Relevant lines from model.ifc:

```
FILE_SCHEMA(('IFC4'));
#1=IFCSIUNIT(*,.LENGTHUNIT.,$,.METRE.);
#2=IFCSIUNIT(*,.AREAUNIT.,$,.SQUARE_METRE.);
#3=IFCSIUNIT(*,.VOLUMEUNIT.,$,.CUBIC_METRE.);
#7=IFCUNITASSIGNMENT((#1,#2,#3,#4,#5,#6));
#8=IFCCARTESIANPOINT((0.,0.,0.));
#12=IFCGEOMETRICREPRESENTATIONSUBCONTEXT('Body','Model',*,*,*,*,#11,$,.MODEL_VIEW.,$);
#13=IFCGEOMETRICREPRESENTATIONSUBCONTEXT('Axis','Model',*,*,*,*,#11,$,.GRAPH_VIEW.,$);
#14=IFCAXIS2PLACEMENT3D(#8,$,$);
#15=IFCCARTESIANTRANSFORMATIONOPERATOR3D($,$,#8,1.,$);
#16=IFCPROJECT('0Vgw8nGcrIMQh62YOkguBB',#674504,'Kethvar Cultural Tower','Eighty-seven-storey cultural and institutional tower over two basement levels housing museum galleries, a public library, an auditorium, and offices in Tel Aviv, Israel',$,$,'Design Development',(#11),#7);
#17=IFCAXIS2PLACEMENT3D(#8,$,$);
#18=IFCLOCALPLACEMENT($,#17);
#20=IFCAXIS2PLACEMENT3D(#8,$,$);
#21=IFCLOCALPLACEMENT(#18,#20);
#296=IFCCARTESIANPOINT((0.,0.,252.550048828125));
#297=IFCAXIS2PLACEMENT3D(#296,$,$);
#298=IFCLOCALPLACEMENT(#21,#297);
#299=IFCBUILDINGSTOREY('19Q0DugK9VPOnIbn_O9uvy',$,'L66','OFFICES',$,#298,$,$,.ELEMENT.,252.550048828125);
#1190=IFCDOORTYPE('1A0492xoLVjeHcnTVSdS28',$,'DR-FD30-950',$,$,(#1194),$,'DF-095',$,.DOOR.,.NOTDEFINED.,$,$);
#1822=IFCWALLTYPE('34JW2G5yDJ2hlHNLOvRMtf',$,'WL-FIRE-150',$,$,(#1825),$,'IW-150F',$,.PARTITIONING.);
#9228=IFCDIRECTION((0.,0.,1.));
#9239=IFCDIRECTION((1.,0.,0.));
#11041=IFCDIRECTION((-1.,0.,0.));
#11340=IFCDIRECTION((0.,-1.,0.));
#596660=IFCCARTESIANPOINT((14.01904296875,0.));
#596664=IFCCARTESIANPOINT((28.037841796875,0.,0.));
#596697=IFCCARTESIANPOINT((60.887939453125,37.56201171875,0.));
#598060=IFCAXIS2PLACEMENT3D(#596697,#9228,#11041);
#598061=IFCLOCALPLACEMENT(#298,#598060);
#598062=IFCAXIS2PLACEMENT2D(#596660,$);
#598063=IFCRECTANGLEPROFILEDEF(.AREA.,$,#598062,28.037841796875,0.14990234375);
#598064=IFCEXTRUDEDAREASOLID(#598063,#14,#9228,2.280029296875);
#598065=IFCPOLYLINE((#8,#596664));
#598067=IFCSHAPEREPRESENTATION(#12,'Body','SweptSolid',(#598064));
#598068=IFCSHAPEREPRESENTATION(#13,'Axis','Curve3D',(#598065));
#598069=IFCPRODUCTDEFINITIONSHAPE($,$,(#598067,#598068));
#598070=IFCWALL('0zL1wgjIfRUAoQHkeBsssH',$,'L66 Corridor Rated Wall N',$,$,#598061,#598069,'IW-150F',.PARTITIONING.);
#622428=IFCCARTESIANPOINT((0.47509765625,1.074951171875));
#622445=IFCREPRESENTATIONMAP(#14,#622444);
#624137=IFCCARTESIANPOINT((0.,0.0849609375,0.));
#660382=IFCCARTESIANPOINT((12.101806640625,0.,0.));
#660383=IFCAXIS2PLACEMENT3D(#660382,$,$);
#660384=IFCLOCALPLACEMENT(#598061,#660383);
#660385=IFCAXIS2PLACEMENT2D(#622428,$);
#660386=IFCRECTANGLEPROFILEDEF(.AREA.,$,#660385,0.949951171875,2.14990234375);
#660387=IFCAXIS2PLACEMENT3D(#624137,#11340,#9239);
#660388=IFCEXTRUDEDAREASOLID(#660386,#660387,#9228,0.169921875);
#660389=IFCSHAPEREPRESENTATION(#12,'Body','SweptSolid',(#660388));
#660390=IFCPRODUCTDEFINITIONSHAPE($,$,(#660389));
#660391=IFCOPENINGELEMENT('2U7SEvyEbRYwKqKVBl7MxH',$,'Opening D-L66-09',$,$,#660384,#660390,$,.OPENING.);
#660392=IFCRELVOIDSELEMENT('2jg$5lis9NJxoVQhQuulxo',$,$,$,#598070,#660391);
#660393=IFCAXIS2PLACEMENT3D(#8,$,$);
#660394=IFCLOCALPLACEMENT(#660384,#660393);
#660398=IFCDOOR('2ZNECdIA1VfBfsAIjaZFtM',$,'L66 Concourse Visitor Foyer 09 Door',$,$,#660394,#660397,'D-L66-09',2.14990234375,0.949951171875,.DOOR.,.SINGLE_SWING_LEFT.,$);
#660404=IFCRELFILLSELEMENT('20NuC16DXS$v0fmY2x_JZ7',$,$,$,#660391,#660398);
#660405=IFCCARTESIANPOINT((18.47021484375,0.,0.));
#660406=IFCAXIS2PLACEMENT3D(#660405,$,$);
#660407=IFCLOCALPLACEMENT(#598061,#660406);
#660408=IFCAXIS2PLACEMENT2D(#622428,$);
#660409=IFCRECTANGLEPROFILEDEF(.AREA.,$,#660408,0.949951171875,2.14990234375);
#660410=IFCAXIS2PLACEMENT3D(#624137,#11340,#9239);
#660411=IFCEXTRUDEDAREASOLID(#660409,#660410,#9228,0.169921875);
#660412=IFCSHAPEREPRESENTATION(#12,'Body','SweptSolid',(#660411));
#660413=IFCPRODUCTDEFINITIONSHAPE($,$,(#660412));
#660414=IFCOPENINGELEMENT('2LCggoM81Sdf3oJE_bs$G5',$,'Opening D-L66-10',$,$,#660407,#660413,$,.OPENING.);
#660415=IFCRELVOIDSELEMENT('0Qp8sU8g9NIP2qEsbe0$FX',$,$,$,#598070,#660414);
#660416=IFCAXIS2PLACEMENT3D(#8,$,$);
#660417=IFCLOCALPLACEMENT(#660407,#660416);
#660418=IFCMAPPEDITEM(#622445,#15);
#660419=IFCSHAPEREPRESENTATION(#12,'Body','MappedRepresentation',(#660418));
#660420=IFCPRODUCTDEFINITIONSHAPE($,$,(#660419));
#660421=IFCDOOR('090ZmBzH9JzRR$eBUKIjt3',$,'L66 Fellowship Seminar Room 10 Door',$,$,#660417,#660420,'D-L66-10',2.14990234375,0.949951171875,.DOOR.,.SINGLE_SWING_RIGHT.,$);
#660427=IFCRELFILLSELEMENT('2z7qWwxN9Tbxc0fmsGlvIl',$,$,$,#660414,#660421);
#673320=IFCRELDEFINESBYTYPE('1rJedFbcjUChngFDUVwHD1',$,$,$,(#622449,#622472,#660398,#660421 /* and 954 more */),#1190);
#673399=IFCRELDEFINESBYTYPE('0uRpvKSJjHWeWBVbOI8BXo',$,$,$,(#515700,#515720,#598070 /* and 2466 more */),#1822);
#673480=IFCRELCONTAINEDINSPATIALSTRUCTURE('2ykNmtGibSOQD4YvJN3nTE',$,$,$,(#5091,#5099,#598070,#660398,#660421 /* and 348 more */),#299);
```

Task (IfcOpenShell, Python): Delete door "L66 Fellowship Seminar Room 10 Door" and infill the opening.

```python
import ifcopenshell
import ifcopenshell.api.feature
import ifcopenshell.api.root
import ifcopenshell.geom
import ifcopenshell.util.shape

model = ifcopenshell.open("model.ifc")
settings = ifcopenshell.geom.settings()


def volume(element):
    """Net volume in cubic metres, openings subtracted."""
    shape = ifcopenshell.geom.create_shape(settings, element)
    return ifcopenshell.util.shape.get_volume(shape.geometry)


door = model.by_guid("090ZmBzH9JzRR$eBUKIjt3")
opening = door.FillsVoids[0].RelatingOpeningElement
wall = opening.VoidsElements[0].RelatingBuildingElement
before = volume(wall)

ifcopenshell.api.root.remove_product(model, product=door)
ifcopenshell.api.feature.remove_feature(model, feature=opening)

after = volume(wall)

print(f"wall volume {before:.3f} -> {after:.3f} m3")

model.write("model_rev.ifc")
```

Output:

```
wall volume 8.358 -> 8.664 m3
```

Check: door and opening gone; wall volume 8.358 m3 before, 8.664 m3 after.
